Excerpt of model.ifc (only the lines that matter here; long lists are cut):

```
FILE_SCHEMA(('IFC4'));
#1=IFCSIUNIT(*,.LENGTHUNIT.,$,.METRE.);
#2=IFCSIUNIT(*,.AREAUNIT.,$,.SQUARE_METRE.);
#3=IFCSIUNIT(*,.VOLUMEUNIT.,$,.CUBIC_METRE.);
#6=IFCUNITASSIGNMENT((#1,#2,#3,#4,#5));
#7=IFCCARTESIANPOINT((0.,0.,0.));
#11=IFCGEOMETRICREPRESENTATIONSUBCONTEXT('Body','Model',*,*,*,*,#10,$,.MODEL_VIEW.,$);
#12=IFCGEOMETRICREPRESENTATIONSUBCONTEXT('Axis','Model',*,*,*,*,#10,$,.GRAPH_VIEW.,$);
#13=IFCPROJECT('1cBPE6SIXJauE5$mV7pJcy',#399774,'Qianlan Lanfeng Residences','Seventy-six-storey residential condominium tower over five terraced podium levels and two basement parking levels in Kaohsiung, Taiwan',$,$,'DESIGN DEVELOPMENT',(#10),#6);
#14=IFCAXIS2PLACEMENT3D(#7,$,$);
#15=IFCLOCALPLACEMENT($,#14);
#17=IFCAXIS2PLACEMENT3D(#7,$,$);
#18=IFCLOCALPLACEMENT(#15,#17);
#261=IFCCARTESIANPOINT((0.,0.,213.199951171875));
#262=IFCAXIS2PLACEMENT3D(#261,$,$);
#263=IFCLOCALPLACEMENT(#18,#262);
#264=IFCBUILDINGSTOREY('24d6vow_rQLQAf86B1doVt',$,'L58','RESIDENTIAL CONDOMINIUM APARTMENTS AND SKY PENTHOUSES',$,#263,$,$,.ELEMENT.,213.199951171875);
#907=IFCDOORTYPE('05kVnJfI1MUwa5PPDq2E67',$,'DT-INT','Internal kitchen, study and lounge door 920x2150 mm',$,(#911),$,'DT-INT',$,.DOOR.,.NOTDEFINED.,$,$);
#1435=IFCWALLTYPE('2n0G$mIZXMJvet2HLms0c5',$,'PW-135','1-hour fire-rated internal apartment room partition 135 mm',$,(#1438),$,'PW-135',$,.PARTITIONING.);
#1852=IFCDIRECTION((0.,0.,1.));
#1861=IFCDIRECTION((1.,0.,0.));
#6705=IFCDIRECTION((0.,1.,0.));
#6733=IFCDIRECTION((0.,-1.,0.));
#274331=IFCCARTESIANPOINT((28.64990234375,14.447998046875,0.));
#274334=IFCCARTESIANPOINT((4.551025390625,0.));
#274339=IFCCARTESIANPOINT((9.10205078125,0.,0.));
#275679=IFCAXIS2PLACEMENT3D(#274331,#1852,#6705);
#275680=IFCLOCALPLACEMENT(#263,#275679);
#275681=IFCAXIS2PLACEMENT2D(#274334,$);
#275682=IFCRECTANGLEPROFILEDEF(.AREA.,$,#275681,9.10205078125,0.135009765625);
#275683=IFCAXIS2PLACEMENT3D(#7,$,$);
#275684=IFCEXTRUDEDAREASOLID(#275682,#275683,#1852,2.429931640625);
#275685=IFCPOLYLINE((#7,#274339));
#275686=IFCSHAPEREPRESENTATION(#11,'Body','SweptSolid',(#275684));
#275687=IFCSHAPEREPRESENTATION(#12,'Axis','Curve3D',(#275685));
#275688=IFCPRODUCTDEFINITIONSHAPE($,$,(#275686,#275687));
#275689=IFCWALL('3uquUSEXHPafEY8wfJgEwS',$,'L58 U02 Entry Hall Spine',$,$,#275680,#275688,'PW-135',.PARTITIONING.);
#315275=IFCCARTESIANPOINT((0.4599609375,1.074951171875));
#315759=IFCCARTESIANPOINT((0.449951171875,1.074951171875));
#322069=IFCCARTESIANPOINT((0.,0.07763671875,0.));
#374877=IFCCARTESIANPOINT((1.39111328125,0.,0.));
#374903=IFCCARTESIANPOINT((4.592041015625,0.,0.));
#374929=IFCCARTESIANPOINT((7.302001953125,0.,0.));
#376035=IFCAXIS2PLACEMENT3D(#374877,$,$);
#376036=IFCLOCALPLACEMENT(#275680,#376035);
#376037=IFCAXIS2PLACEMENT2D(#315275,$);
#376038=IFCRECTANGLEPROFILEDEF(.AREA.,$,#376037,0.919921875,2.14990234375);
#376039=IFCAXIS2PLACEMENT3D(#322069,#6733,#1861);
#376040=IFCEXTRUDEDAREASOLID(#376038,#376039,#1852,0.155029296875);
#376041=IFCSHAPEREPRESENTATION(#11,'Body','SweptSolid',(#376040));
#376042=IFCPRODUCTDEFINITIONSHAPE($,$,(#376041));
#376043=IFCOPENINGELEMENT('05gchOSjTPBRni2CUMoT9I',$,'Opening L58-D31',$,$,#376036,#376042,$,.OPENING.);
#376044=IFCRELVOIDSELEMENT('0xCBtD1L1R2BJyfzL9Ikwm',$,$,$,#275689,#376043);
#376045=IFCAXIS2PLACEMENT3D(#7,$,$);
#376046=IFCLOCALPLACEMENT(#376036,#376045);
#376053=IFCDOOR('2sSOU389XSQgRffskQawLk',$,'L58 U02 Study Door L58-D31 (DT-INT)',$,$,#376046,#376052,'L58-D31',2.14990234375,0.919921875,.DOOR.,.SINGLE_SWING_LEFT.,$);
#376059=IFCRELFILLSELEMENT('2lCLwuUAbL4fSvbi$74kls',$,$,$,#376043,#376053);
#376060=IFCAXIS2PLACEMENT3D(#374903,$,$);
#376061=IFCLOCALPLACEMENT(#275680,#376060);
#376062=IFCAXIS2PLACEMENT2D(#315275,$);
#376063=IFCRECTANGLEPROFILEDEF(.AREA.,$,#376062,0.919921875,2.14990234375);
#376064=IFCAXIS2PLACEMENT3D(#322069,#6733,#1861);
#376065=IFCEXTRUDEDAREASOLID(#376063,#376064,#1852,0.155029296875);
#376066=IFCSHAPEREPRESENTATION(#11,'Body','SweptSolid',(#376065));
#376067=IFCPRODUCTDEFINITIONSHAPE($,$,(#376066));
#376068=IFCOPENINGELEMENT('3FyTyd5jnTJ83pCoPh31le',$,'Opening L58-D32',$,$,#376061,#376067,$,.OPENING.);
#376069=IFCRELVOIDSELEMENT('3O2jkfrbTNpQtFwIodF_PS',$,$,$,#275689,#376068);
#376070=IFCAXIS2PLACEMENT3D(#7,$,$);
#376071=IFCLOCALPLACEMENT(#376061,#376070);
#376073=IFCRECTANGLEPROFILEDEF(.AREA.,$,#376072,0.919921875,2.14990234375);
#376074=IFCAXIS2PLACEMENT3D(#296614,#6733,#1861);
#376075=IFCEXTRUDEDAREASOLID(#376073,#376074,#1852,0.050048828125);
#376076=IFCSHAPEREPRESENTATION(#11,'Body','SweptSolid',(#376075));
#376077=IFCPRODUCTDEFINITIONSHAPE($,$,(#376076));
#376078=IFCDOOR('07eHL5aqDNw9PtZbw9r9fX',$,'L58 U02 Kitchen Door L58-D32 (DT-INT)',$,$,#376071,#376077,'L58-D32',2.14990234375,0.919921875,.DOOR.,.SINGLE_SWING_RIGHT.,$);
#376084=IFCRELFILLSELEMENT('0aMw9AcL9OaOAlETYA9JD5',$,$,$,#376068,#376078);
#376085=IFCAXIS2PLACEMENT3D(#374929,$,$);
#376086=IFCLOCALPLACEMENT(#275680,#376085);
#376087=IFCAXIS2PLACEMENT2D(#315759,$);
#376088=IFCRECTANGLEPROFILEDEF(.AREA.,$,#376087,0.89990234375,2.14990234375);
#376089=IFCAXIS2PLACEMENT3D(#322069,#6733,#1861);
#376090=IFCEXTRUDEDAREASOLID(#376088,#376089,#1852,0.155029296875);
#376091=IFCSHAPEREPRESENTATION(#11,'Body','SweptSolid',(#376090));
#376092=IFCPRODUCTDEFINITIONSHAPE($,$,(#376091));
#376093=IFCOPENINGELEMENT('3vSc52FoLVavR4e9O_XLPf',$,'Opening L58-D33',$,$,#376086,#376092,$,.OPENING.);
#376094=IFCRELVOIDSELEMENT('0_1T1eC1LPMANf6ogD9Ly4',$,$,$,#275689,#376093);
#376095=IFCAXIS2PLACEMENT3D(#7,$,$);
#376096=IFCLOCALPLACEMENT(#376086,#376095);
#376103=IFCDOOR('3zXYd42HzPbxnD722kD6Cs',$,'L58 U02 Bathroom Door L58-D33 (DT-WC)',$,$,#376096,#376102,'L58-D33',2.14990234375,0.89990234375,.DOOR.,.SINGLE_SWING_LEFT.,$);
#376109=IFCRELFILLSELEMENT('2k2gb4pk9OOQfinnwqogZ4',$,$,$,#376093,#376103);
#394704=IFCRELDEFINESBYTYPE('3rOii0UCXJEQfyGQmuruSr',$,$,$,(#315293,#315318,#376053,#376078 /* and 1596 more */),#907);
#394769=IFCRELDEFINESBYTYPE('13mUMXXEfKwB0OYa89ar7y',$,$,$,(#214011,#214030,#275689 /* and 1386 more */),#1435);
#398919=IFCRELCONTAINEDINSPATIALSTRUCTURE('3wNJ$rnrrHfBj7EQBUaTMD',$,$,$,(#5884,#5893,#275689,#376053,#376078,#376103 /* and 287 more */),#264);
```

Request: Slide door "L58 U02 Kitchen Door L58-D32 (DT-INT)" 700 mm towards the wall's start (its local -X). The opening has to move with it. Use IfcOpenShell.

```python
import ifcopenshell
import ifcopenshell.api.geometry
import ifcopenshell.util.placement
import ifcopenshell.util.unit

model = ifcopenshell.open("model.ifc")
unit_scale = ifcopenshell.util.unit.calculate_unit_scale(model)

door = model.by_id(376078)
opening = door.FillsVoids[0].RelatingOpeningElement
wall = opening.VoidsElements[0].RelatingBuildingElement

wall_matrix = ifcopenshell.util.placement.get_local_placement(wall.ObjectPlacement)
shift = wall_matrix[:3, 0] * -0.7 / unit_scale
before = ifcopenshell.util.placement.get_local_placement(door.ObjectPlacement)[:3, 3].copy()

# The door is placed relative to its opening, so it follows when the opening moves.
matrix = ifcopenshell.util.placement.get_local_placement(opening.ObjectPlacement)
matrix[:3, 3] += shift
ifcopenshell.api.geometry.edit_object_placement(
    model, product=opening, matrix=matrix, is_si=False, should_transform_children=True
)

after = ifcopenshell.util.placement.get_local_placement(door.ObjectPlacement)[:3, 3]
print("door moved by", (after - before).round(3) + 0.0)

model.write("model_edited.ifc")
```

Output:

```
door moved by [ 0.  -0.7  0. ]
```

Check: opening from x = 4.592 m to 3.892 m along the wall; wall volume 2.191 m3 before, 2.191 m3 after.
